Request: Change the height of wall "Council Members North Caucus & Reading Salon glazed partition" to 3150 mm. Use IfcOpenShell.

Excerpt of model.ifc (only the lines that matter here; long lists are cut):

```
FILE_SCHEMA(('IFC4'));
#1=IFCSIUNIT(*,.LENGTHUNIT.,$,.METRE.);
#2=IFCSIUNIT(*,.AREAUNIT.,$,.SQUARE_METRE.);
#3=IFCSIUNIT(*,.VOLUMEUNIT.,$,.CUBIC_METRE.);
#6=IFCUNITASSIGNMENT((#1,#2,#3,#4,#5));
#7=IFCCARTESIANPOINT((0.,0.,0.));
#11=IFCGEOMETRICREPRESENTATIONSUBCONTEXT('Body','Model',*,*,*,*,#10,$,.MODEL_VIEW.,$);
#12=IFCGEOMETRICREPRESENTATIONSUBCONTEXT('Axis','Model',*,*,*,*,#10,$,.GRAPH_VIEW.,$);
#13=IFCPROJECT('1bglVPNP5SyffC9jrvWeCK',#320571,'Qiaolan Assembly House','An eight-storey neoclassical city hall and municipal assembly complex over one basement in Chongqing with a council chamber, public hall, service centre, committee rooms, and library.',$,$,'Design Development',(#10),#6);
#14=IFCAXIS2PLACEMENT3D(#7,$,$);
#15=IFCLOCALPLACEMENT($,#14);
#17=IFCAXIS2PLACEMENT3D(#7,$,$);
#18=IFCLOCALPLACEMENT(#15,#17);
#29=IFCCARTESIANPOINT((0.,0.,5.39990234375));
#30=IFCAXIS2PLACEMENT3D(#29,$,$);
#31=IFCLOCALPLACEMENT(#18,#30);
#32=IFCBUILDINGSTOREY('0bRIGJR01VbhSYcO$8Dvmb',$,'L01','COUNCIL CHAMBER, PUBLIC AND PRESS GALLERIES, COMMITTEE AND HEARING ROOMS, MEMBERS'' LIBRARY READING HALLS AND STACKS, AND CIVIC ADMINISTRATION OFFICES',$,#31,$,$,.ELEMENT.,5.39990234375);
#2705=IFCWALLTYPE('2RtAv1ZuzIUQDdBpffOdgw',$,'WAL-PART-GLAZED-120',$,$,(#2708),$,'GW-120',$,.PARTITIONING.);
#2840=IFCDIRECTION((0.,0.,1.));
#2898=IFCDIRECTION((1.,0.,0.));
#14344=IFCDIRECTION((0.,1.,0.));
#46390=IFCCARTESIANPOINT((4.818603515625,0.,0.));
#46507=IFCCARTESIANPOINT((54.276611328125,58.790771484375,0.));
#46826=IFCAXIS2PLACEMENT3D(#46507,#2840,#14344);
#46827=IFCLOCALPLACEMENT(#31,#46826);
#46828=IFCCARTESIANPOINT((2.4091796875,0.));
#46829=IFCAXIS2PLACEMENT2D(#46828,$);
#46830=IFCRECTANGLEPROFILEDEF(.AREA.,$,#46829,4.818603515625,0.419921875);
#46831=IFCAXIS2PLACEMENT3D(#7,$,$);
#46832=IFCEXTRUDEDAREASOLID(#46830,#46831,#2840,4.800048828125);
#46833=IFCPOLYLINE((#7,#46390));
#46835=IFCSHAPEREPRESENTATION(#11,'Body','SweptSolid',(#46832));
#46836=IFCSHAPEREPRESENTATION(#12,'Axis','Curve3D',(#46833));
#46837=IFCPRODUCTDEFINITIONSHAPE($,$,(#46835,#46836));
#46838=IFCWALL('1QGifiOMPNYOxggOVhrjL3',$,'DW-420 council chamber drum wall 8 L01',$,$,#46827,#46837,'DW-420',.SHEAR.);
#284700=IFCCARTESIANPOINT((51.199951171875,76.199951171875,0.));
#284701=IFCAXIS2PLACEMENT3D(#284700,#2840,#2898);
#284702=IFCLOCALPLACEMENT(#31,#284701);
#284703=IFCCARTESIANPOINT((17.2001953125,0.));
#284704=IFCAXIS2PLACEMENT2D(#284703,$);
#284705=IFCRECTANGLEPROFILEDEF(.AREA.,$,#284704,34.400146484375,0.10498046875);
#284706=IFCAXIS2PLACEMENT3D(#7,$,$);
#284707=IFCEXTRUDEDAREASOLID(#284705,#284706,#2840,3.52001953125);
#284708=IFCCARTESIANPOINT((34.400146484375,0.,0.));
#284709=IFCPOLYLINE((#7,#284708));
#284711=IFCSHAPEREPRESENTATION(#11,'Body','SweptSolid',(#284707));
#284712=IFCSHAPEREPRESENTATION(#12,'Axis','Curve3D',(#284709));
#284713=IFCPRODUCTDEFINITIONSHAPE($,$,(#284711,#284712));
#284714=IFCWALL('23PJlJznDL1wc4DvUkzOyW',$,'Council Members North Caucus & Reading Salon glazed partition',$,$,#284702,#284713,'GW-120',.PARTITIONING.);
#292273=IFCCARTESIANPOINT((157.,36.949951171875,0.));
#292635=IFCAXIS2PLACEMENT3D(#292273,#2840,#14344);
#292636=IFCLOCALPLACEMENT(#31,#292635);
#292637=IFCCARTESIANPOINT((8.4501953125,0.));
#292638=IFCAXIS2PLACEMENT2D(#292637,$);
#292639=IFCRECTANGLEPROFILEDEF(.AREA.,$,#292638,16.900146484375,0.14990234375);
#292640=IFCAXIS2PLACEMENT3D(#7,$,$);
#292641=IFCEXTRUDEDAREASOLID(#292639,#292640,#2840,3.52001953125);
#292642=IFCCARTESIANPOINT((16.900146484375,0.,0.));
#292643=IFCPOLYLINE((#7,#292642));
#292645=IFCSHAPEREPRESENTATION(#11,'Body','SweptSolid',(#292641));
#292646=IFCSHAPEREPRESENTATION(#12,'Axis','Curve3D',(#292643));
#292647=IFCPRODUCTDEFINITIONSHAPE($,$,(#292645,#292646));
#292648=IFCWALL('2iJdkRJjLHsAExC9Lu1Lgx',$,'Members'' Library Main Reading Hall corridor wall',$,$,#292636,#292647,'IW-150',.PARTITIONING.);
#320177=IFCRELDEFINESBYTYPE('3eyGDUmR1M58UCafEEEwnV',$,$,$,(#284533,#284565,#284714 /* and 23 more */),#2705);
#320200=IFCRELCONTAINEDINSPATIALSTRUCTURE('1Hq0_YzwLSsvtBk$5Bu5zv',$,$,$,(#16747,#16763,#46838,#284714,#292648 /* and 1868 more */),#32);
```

```python
import ifcopenshell
import ifcopenshell.geom
import ifcopenshell.util.representation
import ifcopenshell.util.shape
import ifcopenshell.util.unit

model = ifcopenshell.open("model.ifc")
unit_scale = ifcopenshell.util.unit.calculate_unit_scale(model)
settings = ifcopenshell.geom.settings()


def volume(element):
    """Net volume in cubic metres, openings subtracted."""
    shape = ifcopenshell.geom.create_shape(settings, element)
    return ifcopenshell.util.shape.get_volume(shape.geometry)


wall = model.by_guid("23PJlJznDL1wc4DvUkzOyW")
before = volume(wall)

body = ifcopenshell.util.representation.get_representation(wall, "Model", "Body")
solid = body.Items[0]
old_height = solid.Depth
solid.Depth = 3.15 / unit_scale
after = volume(wall)

print(f"height {old_height:g} -> {solid.Depth:g}, volume {before:.3f} -> {after:.3f} m3")

model.write("model_updated.ifc")
```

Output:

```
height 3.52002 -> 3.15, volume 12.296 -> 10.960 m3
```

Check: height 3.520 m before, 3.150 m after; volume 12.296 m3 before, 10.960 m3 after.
